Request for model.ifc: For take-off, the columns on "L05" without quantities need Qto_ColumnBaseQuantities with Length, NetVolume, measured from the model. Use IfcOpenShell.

First a look at what the model holds.

```python
import ifcopenshell
import ifcopenshell.util.element
import ifcopenshell.util.unit

model = ifcopenshell.open("model.ifc")
print(model.schema)
for unit_type in ("LENGTHUNIT", "AREAUNIT", "VOLUMEUNIT"):
    print(unit_type, ifcopenshell.util.unit.calculate_unit_scale(model, unit_type))
storey = next(s for s in model.by_type("IfcBuildingStorey") if s.Name == "L05")
columns = [e for e in ifcopenshell.util.element.get_decomposition(storey) if e.is_a("IfcColumn")]
for e in sorted(columns, key=lambda e: e.id()):
    print(e.id(), e.is_a(), e.Name, list(ifcopenshell.util.element.get_psets(e, qtos_only=True)), sep=" | ")
```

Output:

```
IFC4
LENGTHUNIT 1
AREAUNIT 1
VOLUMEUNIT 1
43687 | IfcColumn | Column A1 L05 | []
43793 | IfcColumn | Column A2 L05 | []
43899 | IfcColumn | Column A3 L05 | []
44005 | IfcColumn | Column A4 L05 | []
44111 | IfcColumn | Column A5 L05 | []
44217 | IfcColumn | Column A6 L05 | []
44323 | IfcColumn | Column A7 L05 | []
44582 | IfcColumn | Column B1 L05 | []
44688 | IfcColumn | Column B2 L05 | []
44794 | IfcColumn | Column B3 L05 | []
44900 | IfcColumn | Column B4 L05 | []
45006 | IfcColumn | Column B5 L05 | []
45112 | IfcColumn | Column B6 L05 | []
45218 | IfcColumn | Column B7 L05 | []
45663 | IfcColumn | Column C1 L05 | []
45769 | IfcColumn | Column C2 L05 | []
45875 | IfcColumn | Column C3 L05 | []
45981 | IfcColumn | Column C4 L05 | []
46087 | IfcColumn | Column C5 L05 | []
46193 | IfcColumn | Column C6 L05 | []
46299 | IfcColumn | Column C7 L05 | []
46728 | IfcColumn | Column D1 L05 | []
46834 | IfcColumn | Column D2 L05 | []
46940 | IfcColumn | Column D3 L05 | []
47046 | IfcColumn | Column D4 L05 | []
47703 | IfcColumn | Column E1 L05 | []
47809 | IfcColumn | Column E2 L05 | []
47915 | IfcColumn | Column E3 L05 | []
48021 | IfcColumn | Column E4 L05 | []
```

```python
import ifcopenshell
import ifcopenshell.api.pset
import ifcopenshell.geom
import ifcopenshell.util.element
import ifcopenshell.util.shape
import ifcopenshell.util.unit

model = ifcopenshell.open("model.ifc")
unit_scale = ifcopenshell.util.unit.calculate_unit_scale(model)
volume_scale = ifcopenshell.util.unit.calculate_unit_scale(model, "VOLUMEUNIT")
settings = ifcopenshell.geom.settings()

storey = next(s for s in model.by_type("IfcBuildingStorey") if s.Name == "L05")
columns = [e for e in ifcopenshell.util.element.get_decomposition(storey) if e.is_a("IfcColumn")]

for e in sorted(columns, key=lambda e: e.id()):
    if ifcopenshell.util.element.get_psets(e, qtos_only=True, should_inherit=False):
        continue
    # Geometry comes back in metres, in the element's own axes.
    shape = ifcopenshell.geom.create_shape(settings, e)
    values = {
        "Length": ifcopenshell.util.shape.get_z(shape.geometry) / unit_scale,
        "NetVolume": ifcopenshell.util.shape.get_volume(shape.geometry) / volume_scale,
    }
    qto = ifcopenshell.api.pset.add_qto(model, product=e, name="Qto_ColumnBaseQuantities")
    ifcopenshell.api.pset.edit_qto(model, qto=qto, properties=values)
    print(e.id(), {k: round(v, 3) for k, v in values.items()})

model.write("model_updated.ifc")
```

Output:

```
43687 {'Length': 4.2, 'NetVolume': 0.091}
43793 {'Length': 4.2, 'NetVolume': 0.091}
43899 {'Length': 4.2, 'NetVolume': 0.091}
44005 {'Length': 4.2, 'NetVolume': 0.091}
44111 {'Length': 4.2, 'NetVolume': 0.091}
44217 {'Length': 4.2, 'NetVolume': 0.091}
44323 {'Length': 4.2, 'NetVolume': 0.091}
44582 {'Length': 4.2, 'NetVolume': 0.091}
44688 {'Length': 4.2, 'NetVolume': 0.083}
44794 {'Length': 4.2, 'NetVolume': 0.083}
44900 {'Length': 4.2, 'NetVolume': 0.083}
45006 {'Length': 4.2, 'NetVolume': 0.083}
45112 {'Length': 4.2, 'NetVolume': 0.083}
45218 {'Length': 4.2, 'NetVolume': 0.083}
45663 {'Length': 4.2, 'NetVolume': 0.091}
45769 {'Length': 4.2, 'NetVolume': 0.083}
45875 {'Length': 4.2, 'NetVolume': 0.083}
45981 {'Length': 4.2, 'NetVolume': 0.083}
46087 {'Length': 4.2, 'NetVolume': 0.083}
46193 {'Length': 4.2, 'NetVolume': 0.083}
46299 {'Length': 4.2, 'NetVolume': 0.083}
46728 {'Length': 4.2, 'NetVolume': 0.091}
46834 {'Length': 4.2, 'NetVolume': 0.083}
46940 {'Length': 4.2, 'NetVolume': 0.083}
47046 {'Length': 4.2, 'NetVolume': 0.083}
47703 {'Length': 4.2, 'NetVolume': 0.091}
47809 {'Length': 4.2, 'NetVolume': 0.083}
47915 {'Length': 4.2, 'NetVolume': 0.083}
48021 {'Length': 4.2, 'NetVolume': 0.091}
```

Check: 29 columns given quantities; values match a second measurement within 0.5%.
